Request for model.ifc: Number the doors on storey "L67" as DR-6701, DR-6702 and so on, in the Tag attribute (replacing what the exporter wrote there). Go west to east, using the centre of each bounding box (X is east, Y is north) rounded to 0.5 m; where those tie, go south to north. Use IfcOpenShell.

First a look at what the model holds.

```python
import ifcopenshell
import ifcopenshell.util.element
import ifcopenshell.util.placement

model = ifcopenshell.open("model.ifc")
print(model.schema)
storey = next(s for s in model.by_type("IfcBuildingStorey") if s.Name == "L67")
doors = [e for e in ifcopenshell.util.element.get_decomposition(storey) if e.is_a("IfcDoor")]
for e in sorted(doors, key=lambda e: e.id()):
    origin = ifcopenshell.util.placement.get_local_placement(e.ObjectPlacement)[:3, 3]
    print(e.id(), e.Tag, e.Name, origin.round(2) + 0.0, sep=" | ")
```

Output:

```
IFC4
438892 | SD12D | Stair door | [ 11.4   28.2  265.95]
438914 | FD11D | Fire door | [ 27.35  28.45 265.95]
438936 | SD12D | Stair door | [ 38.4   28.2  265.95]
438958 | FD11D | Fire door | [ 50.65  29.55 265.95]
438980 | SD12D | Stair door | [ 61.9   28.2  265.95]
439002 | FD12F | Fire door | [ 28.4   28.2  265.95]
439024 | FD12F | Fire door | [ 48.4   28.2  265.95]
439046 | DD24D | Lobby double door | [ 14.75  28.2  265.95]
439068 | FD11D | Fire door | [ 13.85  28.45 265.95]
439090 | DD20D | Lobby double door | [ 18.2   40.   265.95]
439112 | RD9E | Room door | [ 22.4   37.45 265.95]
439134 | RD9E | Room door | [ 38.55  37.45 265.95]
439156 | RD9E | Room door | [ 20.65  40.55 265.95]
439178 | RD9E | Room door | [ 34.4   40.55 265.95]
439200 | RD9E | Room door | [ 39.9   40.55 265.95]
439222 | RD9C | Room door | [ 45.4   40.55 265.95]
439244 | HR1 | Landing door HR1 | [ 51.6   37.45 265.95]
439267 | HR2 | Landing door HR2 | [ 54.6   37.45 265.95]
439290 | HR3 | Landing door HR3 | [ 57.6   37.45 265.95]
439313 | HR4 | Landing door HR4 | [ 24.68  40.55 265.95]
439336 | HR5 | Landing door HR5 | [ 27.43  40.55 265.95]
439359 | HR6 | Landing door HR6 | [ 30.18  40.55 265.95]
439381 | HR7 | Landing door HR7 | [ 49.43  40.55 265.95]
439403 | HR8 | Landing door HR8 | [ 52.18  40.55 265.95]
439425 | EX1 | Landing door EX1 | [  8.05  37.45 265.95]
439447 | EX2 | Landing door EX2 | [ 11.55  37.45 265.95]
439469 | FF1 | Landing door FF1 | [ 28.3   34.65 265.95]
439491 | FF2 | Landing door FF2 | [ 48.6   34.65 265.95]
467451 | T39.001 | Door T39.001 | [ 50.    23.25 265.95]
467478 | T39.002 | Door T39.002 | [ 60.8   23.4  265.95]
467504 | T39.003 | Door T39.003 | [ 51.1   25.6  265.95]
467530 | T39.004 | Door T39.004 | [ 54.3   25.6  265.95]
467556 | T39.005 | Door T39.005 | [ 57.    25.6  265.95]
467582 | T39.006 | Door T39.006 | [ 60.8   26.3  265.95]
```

```python
import ifcopenshell
import ifcopenshell.geom
import ifcopenshell.util.element
import ifcopenshell.util.shape

model = ifcopenshell.open("model.ifc")
settings = ifcopenshell.geom.settings()
settings.set("use-world-coords", True)


def centre(element):
    shape = ifcopenshell.geom.create_shape(settings, element)
    return ifcopenshell.util.shape.get_bbox_centroid(shape.geometry)


storey = next(s for s in model.by_type("IfcBuildingStorey") if s.Name == "L67")
doors = [e for e in ifcopenshell.util.element.get_decomposition(storey) if e.is_a("IfcDoor")]

# Insertion points can sit at a corner or the storey origin, so sort by the geometry (in metres).
centres = {e: centre(e) for e in doors}
doors.sort(key=lambda e: (round(centres[e][0] / 0.5), centres[e][1]))

for i, e in enumerate(doors, start=1):
    number = f"DR-67{i:02d}"
    e.Tag = number
    print(e.id(), number)

model.write("model_edited.ifc")
```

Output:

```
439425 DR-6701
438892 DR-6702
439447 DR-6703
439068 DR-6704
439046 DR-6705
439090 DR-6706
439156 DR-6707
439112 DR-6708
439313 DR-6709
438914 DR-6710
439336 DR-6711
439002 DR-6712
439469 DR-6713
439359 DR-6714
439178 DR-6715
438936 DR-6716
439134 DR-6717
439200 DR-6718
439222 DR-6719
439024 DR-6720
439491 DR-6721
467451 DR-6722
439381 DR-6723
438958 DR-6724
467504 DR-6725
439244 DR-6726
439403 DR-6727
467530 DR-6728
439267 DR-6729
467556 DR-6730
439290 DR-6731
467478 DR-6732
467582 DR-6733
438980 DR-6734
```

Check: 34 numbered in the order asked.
